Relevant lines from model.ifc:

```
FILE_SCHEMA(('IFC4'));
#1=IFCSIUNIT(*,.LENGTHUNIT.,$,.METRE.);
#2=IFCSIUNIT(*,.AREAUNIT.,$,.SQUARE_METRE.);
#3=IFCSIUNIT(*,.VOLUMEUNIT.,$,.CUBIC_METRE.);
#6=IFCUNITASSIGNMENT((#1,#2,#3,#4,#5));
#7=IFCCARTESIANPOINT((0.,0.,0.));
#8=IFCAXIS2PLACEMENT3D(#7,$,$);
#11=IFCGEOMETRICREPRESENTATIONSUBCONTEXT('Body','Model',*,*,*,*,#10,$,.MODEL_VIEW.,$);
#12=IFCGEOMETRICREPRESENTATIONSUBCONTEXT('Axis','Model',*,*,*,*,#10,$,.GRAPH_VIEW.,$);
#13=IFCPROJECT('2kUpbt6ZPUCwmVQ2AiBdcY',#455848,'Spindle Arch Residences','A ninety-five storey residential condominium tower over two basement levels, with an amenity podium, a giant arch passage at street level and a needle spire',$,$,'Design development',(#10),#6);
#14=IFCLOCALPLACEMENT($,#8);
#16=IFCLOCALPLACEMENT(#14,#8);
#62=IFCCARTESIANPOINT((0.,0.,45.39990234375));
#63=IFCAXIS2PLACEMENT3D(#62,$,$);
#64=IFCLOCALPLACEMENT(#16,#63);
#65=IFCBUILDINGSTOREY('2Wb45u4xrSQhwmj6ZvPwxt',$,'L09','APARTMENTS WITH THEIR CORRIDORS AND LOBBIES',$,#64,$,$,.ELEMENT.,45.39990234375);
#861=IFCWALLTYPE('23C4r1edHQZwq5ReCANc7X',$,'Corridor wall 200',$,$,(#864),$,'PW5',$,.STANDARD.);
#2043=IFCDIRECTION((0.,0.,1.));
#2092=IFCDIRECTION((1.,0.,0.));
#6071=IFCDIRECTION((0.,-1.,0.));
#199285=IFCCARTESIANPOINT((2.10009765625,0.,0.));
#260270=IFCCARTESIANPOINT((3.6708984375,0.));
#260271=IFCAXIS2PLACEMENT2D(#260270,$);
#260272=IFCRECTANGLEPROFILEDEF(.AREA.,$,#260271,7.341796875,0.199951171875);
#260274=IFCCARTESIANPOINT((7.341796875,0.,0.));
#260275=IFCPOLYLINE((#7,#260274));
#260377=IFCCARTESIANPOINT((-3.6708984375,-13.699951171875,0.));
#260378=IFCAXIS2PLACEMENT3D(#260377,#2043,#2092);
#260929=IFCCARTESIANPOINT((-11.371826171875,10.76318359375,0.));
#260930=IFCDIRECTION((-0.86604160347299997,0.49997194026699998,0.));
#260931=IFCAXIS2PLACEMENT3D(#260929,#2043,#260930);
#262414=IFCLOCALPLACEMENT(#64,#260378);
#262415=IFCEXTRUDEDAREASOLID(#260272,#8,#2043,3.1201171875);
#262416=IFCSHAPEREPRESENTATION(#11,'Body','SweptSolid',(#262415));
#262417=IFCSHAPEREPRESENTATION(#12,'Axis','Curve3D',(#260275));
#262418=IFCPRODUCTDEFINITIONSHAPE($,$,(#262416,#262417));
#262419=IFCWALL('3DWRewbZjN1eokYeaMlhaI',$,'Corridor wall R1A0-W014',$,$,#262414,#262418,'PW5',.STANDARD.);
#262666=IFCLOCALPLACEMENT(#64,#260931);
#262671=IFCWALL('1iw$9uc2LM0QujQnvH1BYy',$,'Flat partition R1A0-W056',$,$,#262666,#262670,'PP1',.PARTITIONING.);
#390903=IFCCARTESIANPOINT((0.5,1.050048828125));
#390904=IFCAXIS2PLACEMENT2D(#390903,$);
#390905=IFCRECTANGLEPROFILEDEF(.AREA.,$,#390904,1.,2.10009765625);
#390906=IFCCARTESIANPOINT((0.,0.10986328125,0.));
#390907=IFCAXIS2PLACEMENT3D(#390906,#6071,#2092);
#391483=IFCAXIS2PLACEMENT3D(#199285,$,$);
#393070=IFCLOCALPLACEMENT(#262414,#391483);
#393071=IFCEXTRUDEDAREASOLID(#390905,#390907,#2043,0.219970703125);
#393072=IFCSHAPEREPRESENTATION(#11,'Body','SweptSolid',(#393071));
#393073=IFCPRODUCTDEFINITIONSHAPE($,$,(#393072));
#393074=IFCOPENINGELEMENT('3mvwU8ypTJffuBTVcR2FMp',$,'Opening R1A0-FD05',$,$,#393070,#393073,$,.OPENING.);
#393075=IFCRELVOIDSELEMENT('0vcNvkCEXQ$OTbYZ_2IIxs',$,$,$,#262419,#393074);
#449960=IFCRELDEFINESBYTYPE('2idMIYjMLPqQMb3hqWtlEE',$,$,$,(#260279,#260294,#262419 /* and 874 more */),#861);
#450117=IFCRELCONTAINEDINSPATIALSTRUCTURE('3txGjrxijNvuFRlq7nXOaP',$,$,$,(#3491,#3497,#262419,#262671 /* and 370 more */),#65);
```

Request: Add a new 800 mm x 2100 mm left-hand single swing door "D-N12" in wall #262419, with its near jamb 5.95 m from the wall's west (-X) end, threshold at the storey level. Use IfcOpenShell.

```python
import numpy as np
import ifcopenshell
import ifcopenshell.api.feature
import ifcopenshell.api.geometry
import ifcopenshell.api.root
import ifcopenshell.api.spatial
import ifcopenshell.geom
import ifcopenshell.util.element
import ifcopenshell.util.placement
import ifcopenshell.util.representation
import ifcopenshell.util.shape
import ifcopenshell.util.unit

model = ifcopenshell.open("model.ifc")
unit_scale = ifcopenshell.util.unit.calculate_unit_scale(model)
settings = ifcopenshell.geom.settings()


def volume(element):
    """Net volume in cubic metres, openings subtracted."""
    shape = ifcopenshell.geom.create_shape(settings, element)
    return ifcopenshell.util.shape.get_volume(shape.geometry)


wall = model.by_guid("3DWRewbZjN1eokYeaMlhaI")
storey = ifcopenshell.util.element.get_container(wall, ifc_class="IfcBuildingStorey")
context = ifcopenshell.util.representation.get_context(model, "Model", "Body", "MODEL_VIEW")
before = volume(wall)

width, height, from_end, sill = 0.8, 2.1, 5.95, 0.0  # metres

# The wall runs along its own X axis, and the end named is its -X end.
wall_shape = ifcopenshell.geom.create_shape(settings, wall)
x, y, z = ifcopenshell.util.shape.get_vertices(wall_shape.geometry).T
start = x.min() + from_end
face, thickness = float(y.min()), float(y.max() - y.min())
wall_matrix = ifcopenshell.util.placement.get_local_placement(wall.ObjectPlacement)
level = ifcopenshell.util.placement.get_local_placement(storey.ObjectPlacement)[2, 3]


def in_wall(x, y):
    """Placement at x, y metres in the wall's axes, at sill height."""
    matrix = wall_matrix.copy()
    matrix[:, 3] = wall_matrix @ np.array([x / unit_scale, y / unit_scale, 0.0, 1.0])
    matrix[2, 3] = level + sill / unit_scale
    return matrix


# Opening: a box that overshoots both wall faces by 50 mm.
opening = ifcopenshell.api.root.create_entity(model, ifc_class="IfcOpeningElement", predefined_type="OPENING")
box = ifcopenshell.api.geometry.add_wall_representation(
    model, context=context, length=width, height=height, thickness=thickness + 0.1
)
ifcopenshell.api.geometry.assign_representation(model, product=opening, representation=box)
ifcopenshell.api.geometry.edit_object_placement(model, product=opening, matrix=in_wall(start, face - 0.05), is_si=False)
ifcopenshell.api.feature.add_feature(model, feature=opening, element=wall)

door = ifcopenshell.api.root.create_entity(model, ifc_class="IfcDoor", name="D-N12", predefined_type="DOOR")
door.OverallWidth, door.OverallHeight = width / unit_scale, height / unit_scale
door.OperationType = "SINGLE_SWING_LEFT"
body = ifcopenshell.api.geometry.add_door_representation(
    model,
    context=context,
    overall_width=door.OverallWidth,
    overall_height=door.OverallHeight,
    operation_type="SINGLE_SWING_LEFT",
    lining_properties={"LiningDepth": thickness / unit_scale, "ThresholdDepth": thickness / unit_scale},
)
ifcopenshell.api.geometry.assign_representation(model, product=door, representation=body)
ifcopenshell.api.spatial.assign_container(model, products=[door], relating_structure=storey)
ifcopenshell.api.feature.add_filling(model, opening=opening, element=door)

# The lining spans the wall, so the door starts at the wall face.
ifcopenshell.api.geometry.edit_object_placement(model, product=door, matrix=in_wall(start, face), is_si=False)

after = volume(wall)

print(f"wall volume {before:.3f} -> {after:.3f} m3")

model.write("model_v2.ifc")
```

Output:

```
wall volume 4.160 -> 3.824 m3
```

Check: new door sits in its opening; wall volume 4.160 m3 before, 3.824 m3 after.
